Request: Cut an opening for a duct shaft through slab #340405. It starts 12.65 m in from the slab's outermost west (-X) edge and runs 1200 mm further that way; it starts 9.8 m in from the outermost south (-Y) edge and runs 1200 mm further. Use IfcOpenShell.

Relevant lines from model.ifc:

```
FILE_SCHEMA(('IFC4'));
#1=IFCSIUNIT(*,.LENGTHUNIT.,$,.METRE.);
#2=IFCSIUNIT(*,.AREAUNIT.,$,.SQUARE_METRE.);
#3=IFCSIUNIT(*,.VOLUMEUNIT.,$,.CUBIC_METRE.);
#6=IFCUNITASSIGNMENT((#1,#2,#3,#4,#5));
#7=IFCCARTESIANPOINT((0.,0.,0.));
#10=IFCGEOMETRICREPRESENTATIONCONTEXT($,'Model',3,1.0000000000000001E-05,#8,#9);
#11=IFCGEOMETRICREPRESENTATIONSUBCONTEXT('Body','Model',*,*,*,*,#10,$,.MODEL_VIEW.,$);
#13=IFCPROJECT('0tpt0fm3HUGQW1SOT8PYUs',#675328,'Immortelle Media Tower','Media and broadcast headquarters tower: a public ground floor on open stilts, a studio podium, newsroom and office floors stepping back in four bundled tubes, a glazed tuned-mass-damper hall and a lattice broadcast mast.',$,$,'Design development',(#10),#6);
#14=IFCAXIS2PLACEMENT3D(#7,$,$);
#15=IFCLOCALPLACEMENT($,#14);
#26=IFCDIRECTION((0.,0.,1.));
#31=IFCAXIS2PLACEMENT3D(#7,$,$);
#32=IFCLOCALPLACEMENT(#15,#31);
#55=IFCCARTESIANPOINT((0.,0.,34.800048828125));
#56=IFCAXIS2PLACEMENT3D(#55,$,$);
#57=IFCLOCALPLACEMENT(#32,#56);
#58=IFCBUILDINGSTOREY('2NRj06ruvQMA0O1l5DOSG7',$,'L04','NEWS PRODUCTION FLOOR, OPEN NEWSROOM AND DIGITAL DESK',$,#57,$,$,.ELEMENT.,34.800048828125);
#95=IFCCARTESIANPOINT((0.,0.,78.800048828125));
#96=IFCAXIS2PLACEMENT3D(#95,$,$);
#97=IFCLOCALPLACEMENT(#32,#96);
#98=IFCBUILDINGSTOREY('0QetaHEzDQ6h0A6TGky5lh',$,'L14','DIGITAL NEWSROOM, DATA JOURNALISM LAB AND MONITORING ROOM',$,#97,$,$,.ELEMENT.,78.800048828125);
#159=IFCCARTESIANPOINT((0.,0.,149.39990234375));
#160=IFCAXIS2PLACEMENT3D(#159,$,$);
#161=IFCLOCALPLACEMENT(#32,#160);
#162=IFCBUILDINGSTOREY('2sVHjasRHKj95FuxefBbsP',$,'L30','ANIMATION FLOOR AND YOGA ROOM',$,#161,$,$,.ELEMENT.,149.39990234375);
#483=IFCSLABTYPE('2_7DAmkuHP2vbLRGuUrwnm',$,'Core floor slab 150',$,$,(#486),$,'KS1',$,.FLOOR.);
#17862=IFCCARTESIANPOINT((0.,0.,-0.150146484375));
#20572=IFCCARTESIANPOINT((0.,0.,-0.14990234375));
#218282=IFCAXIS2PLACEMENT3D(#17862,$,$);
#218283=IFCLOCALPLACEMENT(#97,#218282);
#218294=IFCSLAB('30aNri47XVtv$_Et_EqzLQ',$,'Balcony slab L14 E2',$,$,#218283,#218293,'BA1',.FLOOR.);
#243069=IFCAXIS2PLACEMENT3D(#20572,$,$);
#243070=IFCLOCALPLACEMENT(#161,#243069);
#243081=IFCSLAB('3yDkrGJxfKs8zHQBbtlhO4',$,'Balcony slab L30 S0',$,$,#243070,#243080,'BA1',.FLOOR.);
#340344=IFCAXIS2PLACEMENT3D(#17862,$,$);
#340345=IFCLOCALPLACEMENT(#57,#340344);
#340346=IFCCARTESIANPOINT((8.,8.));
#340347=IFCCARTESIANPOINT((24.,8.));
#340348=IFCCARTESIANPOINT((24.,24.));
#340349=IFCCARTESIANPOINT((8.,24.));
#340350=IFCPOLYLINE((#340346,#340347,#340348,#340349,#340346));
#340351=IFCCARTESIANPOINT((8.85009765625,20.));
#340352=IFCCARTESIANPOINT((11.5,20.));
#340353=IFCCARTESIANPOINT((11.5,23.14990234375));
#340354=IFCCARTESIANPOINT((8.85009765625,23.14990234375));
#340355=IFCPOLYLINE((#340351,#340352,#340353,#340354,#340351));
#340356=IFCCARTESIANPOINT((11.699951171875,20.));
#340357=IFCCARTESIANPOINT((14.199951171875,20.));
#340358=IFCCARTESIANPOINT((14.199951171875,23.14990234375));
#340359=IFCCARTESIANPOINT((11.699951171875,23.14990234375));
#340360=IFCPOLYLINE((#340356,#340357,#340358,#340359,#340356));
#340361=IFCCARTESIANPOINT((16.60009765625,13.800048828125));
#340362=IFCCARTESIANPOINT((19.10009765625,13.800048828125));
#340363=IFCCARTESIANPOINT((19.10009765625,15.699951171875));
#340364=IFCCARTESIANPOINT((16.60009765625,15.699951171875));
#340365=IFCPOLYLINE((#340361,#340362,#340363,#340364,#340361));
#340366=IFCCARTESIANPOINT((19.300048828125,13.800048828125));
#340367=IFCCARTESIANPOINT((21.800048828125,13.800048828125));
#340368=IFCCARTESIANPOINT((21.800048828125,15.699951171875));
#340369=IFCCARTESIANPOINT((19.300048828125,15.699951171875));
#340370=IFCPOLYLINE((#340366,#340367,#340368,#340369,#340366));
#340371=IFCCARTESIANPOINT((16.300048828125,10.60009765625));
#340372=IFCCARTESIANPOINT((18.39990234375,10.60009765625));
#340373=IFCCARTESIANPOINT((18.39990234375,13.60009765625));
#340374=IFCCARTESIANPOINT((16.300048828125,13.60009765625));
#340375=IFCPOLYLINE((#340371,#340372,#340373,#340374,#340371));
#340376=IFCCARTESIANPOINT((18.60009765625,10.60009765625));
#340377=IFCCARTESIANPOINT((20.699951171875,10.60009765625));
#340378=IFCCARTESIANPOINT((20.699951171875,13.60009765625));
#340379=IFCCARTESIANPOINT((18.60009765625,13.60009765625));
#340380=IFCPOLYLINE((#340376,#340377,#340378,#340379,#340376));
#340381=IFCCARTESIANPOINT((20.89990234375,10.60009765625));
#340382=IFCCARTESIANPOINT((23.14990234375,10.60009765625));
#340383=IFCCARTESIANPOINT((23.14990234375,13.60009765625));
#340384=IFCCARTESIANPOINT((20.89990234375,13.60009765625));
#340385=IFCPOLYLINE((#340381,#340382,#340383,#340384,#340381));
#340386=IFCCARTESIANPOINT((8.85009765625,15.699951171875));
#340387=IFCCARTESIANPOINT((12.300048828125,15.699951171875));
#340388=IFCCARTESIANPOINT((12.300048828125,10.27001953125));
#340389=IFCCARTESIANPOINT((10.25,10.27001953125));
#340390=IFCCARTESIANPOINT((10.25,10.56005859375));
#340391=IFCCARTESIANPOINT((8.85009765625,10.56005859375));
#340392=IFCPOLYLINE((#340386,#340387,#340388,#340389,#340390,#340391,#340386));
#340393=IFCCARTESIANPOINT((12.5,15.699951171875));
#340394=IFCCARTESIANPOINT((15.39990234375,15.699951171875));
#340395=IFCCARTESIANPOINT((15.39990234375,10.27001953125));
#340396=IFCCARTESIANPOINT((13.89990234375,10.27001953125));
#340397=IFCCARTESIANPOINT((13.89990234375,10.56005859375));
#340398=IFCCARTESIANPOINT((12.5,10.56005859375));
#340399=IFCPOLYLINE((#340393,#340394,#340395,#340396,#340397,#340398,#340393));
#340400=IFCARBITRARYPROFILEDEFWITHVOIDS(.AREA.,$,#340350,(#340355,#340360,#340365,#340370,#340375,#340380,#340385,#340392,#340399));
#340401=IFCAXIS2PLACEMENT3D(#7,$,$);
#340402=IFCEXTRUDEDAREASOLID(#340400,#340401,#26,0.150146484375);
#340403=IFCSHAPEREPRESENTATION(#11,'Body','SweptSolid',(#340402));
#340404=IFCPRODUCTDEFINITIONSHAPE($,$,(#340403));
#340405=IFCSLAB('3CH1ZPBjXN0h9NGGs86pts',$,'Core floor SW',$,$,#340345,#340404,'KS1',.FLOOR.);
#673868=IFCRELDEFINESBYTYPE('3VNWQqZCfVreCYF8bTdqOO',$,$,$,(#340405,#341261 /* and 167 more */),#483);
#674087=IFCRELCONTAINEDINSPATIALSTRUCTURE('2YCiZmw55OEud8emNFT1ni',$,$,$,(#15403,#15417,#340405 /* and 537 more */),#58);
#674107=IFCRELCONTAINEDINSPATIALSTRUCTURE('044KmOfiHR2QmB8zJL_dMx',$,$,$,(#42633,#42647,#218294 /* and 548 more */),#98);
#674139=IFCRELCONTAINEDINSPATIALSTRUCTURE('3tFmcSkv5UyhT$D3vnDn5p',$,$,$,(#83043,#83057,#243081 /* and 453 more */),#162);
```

```python
import numpy as np
import ifcopenshell
import ifcopenshell.api.feature
import ifcopenshell.api.geometry
import ifcopenshell.api.root
import ifcopenshell.geom
import ifcopenshell.util.placement
import ifcopenshell.util.representation
import ifcopenshell.util.shape
import ifcopenshell.util.unit

model = ifcopenshell.open("model.ifc")
unit_scale = ifcopenshell.util.unit.calculate_unit_scale(model)
settings = ifcopenshell.geom.settings()


def volume(element):
    """Net volume in cubic metres, openings subtracted."""
    shape = ifcopenshell.geom.create_shape(settings, element)
    return ifcopenshell.util.shape.get_volume(shape.geometry)


slab = model.by_guid("3CH1ZPBjXN0h9NGGs86pts")
before = volume(slab)

# Extent in the slab's own axes, in metres. The edges named are its -X and -Y sides.
slab_shape = ifcopenshell.geom.create_shape(settings, slab)
vertices = ifcopenshell.util.shape.get_vertices(slab_shape.geometry)
x_min, y_min, bottom = vertices.min(axis=0)
top = vertices[:, 2].max()

opening = ifcopenshell.api.root.create_entity(model, ifc_class="IfcOpeningElement", name="Duct shaft opening", predefined_type="OPENING")
context = ifcopenshell.util.representation.get_context(model, "Model", "Body", "MODEL_VIEW")
width, depth = 1.2, 1.2
outline = [(0.0, 0.0), (width, 0.0), (width, depth), (0.0, depth), (0.0, 0.0)]
# Overshoot both faces by 50 mm so the cut is clean.
shape = ifcopenshell.api.geometry.add_slab_representation(
    model, context=context, depth=top - bottom + 0.1, polyline=outline
)
ifcopenshell.api.geometry.assign_representation(model, product=opening, representation=shape)

matrix = ifcopenshell.util.placement.get_local_placement(slab.ObjectPlacement)
matrix[:, 3] = matrix @ np.append(np.array([x_min + 12.65, y_min + 9.8, bottom - 0.05]) / unit_scale, 1.0)
ifcopenshell.api.geometry.edit_object_placement(model, product=opening, matrix=matrix, is_si=False)
ifcopenshell.api.feature.add_feature(model, feature=opening, element=slab)

after = volume(slab)

print(f"slab volume {before:.3f} -> {after:.3f} m3")

model.write("model-out.ifc")
```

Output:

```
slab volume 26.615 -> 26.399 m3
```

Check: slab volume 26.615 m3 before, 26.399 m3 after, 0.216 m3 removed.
